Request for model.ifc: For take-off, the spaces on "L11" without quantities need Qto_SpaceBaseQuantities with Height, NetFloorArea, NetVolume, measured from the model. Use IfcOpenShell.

First a look at what the model holds.

```python
import ifcopenshell
import ifcopenshell.util.element
import ifcopenshell.util.unit

model = ifcopenshell.open("model.ifc")
print(model.schema)
for unit_type in ("LENGTHUNIT", "AREAUNIT", "VOLUMEUNIT"):
    print(unit_type, ifcopenshell.util.unit.calculate_unit_scale(model, unit_type))
storey = next(s for s in model.by_type("IfcBuildingStorey") if s.Name == "L11")
spaces = [e for e in ifcopenshell.util.element.get_decomposition(storey) if e.is_a("IfcSpace")]
for e in sorted(spaces, key=lambda e: e.id()):
    print(e.id(), e.is_a(), e.Name, list(ifcopenshell.util.element.get_psets(e, qtos_only=True)), sep=" | ")
```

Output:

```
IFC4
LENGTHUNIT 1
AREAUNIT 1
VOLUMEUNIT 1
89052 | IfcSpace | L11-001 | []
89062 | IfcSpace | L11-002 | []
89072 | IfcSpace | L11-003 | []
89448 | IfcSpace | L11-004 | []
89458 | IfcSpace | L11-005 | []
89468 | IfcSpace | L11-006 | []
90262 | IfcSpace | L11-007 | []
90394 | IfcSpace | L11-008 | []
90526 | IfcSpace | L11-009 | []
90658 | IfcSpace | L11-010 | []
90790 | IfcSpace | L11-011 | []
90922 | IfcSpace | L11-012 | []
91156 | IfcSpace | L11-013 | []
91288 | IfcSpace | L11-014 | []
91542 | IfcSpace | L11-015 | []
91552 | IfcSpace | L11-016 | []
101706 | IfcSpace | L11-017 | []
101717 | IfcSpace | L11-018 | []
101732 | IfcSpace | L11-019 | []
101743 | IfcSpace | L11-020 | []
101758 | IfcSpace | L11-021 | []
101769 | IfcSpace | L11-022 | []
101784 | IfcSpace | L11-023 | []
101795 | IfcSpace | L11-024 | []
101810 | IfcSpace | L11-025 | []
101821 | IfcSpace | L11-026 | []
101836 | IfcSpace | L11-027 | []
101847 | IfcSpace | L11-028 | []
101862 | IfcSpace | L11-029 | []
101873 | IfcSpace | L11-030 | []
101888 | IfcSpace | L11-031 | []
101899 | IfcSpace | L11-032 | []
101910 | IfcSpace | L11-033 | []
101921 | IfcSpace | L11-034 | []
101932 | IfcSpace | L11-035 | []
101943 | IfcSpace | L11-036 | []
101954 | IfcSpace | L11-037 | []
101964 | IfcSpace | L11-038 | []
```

```python
import ifcopenshell
import ifcopenshell.api.pset
import ifcopenshell.geom
import ifcopenshell.util.element
import ifcopenshell.util.shape
import ifcopenshell.util.unit

model = ifcopenshell.open("model.ifc")
unit_scale = ifcopenshell.util.unit.calculate_unit_scale(model)
area_scale = ifcopenshell.util.unit.calculate_unit_scale(model, "AREAUNIT")
volume_scale = ifcopenshell.util.unit.calculate_unit_scale(model, "VOLUMEUNIT")
settings = ifcopenshell.geom.settings()

storey = next(s for s in model.by_type("IfcBuildingStorey") if s.Name == "L11")
spaces = [e for e in ifcopenshell.util.element.get_decomposition(storey) if e.is_a("IfcSpace")]

for e in sorted(spaces, key=lambda e: e.id()):
    if ifcopenshell.util.element.get_psets(e, qtos_only=True, should_inherit=False):
        continue
    # Geometry comes back in metres, in the element's own axes.
    shape = ifcopenshell.geom.create_shape(settings, e)
    values = {
        "Height": ifcopenshell.util.shape.get_z(shape.geometry) / unit_scale,
        "NetFloorArea": ifcopenshell.util.shape.get_footprint_area(shape.geometry) / area_scale,
        "NetVolume": ifcopenshell.util.shape.get_volume(shape.geometry) / volume_scale,
    }
    qto = ifcopenshell.api.pset.add_qto(model, product=e, name="Qto_SpaceBaseQuantities")
    ifcopenshell.api.pset.edit_qto(model, qto=qto, properties=values)
    print(e.id(), {k: round(v, 3) for k, v in values.items()})

model.write("model_v2.ifc")
```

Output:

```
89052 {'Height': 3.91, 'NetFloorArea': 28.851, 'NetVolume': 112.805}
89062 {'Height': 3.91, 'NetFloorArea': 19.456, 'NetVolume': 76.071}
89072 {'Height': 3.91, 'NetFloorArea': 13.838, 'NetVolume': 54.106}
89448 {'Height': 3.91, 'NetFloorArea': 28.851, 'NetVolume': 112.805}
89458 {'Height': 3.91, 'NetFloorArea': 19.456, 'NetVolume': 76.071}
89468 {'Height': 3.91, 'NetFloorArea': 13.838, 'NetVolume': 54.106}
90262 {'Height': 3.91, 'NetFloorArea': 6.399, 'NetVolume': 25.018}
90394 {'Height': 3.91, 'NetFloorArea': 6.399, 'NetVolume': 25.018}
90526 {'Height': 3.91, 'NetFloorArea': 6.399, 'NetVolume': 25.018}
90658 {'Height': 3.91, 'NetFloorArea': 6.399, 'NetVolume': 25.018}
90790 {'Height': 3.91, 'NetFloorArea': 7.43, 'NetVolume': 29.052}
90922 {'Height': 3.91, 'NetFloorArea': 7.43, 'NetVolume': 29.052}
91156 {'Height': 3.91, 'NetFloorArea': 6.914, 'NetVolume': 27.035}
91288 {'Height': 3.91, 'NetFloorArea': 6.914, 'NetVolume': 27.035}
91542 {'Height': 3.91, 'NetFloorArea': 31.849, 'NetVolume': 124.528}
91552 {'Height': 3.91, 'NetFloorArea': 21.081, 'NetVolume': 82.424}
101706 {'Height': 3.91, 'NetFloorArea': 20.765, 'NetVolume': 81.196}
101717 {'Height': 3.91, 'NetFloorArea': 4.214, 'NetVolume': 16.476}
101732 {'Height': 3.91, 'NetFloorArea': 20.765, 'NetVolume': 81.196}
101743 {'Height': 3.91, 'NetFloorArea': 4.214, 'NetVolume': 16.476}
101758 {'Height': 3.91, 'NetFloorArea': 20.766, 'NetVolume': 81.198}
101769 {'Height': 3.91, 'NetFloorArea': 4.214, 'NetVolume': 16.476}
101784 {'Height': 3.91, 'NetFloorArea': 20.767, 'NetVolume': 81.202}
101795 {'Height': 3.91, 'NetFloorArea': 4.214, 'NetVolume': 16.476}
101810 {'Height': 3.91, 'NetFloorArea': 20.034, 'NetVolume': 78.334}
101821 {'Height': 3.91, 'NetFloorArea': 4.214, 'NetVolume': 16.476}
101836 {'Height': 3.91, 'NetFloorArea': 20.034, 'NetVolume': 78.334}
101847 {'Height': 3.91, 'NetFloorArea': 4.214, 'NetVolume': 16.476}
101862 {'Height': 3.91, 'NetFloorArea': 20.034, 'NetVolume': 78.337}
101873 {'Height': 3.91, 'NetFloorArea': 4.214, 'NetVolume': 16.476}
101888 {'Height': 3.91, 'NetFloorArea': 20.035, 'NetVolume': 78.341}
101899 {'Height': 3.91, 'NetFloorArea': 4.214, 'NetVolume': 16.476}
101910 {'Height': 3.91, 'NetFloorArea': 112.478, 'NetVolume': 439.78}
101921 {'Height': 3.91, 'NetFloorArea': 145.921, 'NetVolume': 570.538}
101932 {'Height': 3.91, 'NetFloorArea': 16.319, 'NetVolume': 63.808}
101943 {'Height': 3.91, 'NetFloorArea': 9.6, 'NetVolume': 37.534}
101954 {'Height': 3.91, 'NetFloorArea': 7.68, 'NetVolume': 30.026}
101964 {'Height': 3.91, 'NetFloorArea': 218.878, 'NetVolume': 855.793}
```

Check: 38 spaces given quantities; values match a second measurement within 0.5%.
